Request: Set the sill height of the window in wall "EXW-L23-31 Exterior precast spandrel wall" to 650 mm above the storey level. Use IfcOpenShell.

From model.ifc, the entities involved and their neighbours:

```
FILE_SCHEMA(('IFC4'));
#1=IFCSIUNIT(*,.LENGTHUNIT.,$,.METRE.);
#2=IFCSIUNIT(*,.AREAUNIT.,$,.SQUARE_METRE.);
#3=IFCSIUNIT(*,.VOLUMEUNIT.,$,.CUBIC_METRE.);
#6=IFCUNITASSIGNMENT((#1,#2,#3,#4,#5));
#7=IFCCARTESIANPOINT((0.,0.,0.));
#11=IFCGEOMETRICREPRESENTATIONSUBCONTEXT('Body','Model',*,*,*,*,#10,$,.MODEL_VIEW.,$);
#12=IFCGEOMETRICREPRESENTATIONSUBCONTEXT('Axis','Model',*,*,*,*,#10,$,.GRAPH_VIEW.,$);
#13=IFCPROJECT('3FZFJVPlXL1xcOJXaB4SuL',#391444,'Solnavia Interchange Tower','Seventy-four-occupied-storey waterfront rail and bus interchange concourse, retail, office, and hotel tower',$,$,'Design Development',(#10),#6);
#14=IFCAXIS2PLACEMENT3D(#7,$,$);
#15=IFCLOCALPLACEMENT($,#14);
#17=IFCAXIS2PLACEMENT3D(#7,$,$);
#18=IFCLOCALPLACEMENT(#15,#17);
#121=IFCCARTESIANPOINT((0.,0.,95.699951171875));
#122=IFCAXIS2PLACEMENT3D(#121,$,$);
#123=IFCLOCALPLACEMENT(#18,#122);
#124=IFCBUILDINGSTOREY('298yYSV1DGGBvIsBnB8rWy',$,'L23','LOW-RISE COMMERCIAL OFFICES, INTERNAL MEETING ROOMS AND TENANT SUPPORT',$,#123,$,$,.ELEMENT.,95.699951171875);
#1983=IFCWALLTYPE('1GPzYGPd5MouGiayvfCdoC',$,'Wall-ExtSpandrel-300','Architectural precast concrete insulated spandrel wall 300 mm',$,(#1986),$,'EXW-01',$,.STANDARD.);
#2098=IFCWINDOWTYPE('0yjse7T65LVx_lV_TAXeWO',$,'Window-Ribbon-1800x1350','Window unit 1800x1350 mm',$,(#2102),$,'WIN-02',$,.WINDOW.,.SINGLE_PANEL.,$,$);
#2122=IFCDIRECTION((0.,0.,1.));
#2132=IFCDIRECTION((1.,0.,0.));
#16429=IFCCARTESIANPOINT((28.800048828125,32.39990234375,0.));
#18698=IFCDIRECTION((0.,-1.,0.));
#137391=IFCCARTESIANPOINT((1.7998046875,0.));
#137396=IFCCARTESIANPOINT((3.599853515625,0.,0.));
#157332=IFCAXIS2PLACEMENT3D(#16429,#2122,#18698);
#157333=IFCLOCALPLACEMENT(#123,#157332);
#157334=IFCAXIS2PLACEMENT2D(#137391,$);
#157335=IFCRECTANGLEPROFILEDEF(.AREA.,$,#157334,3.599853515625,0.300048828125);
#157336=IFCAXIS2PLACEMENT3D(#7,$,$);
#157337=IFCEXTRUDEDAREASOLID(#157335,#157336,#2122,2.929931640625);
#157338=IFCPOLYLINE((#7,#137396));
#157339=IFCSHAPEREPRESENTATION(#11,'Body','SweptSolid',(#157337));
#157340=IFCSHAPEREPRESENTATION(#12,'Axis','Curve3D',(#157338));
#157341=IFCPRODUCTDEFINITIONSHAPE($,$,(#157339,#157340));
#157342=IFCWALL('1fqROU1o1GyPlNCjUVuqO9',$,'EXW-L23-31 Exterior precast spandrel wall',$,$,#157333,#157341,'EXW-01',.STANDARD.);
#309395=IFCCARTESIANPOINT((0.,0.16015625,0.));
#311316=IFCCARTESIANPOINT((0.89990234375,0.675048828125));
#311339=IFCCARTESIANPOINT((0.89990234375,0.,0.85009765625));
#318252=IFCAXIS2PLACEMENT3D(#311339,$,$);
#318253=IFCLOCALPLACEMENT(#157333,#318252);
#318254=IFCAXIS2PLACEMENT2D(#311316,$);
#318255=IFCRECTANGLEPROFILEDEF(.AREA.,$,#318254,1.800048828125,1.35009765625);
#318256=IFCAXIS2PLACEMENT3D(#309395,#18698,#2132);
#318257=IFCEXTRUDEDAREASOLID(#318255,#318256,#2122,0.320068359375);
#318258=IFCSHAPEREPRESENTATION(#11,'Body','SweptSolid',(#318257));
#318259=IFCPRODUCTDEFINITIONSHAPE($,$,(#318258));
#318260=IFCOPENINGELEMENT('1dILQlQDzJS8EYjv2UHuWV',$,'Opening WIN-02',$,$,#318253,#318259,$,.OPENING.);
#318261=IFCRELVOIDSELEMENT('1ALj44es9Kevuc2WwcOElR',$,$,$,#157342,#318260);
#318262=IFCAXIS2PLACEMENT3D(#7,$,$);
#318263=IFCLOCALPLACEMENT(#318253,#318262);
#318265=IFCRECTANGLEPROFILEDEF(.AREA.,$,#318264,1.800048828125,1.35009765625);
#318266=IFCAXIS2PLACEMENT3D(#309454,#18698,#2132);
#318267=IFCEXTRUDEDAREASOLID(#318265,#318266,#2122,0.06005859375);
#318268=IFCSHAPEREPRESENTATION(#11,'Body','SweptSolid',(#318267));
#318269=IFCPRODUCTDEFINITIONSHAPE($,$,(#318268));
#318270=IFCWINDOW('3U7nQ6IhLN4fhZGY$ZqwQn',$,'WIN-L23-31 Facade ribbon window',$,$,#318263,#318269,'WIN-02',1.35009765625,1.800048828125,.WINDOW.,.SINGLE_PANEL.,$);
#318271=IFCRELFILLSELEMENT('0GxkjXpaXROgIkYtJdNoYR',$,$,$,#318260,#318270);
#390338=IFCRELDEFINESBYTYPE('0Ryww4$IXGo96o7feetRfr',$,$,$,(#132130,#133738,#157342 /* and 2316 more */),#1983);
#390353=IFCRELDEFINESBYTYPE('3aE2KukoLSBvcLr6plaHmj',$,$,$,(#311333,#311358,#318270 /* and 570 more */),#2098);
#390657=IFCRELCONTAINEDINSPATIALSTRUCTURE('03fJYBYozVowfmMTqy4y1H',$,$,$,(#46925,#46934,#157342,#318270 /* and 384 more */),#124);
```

```python
import numpy as np
import ifcopenshell
import ifcopenshell.api.geometry
import ifcopenshell.geom
import ifcopenshell.util.element
import ifcopenshell.util.placement
import ifcopenshell.util.shape
import ifcopenshell.util.unit

model = ifcopenshell.open("model.ifc")
unit_scale = ifcopenshell.util.unit.calculate_unit_scale(model)

window = model.by_guid("3U7nQ6IhLN4fhZGY$ZqwQn")
opening = window.FillsVoids[0].RelatingOpeningElement
storey = ifcopenshell.util.element.get_container(window, ifc_class="IfcBuildingStorey")
level = ifcopenshell.util.placement.get_local_placement(storey.ObjectPlacement)[2, 3]

# The opening's origin need not be at the sill, so measure its lowest point.
shape = ifcopenshell.geom.create_shape(ifcopenshell.geom.settings(), opening)
bottom = ifcopenshell.util.shape.get_shape_bottom_elevation(shape, shape.geometry) / unit_scale
dz = level + 0.65 - bottom

shift = np.array([0.0, 0.0, dz])
# The window is placed relative to its opening, so it follows when the opening moves.
matrix = ifcopenshell.util.placement.get_local_placement(opening.ObjectPlacement)
matrix[:3, 3] += shift
ifcopenshell.api.geometry.edit_object_placement(
    model, product=opening, matrix=matrix, is_si=False, should_transform_children=True
)

print(f"moved by {dz * unit_scale:+.3f} m")

model.write("model-out.ifc")
```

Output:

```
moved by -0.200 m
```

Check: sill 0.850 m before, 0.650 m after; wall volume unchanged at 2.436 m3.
